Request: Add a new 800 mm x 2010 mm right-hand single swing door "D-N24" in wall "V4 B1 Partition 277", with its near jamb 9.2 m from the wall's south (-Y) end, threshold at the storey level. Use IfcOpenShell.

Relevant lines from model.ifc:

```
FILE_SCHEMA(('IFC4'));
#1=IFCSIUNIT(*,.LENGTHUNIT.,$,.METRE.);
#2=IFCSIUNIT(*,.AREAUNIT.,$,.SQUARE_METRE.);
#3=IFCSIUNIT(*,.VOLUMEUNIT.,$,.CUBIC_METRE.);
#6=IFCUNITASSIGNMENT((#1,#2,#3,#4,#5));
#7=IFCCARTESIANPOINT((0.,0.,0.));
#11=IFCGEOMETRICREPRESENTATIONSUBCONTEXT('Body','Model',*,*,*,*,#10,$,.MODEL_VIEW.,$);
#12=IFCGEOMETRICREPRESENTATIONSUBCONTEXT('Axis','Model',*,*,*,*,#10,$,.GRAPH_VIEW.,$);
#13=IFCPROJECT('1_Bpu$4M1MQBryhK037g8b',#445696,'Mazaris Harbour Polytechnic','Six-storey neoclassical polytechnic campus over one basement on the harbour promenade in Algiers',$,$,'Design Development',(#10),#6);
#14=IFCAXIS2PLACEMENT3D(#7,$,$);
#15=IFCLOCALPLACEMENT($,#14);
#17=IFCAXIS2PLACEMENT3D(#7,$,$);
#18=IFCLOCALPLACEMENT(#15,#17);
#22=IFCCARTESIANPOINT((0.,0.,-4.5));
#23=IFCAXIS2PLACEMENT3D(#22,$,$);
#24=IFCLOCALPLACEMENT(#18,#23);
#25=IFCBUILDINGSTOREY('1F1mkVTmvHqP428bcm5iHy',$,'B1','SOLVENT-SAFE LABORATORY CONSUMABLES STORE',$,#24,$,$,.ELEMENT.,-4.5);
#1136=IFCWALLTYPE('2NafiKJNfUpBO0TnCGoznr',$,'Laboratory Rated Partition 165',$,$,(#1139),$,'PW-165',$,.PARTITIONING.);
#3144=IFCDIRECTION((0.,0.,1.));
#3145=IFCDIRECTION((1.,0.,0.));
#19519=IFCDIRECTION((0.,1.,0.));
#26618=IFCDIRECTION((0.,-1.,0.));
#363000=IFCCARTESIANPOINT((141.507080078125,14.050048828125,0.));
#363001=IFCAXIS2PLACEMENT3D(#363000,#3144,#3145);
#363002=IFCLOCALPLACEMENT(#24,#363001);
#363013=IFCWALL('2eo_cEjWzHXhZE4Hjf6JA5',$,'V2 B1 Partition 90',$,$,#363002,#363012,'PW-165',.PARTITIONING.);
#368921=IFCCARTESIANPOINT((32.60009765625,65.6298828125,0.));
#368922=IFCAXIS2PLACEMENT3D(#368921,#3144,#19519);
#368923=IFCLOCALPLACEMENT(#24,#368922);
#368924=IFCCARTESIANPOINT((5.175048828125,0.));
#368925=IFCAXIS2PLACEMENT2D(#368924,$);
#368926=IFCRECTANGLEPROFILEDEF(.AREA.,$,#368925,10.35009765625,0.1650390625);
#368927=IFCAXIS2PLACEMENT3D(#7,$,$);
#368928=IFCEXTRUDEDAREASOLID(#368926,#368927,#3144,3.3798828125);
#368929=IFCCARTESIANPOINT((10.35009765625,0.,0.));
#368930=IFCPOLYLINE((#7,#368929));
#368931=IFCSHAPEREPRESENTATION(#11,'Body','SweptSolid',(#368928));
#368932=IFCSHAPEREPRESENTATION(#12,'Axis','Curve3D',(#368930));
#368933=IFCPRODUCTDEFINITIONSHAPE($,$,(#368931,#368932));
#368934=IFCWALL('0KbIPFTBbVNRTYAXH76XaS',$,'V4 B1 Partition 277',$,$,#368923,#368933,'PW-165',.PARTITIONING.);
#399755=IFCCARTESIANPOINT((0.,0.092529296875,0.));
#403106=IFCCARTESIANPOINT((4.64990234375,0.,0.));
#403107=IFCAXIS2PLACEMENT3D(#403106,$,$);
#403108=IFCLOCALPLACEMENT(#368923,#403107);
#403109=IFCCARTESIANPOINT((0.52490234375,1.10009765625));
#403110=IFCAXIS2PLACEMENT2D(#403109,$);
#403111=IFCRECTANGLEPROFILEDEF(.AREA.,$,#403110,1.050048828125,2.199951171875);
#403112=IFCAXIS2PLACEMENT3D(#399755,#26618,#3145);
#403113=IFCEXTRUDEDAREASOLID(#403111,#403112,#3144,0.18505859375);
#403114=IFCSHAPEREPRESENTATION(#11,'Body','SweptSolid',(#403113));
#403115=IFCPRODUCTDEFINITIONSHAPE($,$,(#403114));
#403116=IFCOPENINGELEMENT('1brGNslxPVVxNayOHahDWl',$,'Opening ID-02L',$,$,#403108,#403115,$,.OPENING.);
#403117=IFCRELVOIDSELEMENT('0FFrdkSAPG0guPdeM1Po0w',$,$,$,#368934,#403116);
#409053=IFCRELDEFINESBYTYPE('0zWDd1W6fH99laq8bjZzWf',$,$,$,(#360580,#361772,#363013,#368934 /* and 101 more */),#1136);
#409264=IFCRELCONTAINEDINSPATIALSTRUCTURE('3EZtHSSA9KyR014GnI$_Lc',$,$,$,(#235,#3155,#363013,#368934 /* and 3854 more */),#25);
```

```python
import numpy as np
import ifcopenshell
import ifcopenshell.api.feature
import ifcopenshell.api.geometry
import ifcopenshell.api.root
import ifcopenshell.api.spatial
import ifcopenshell.geom
import ifcopenshell.util.element
import ifcopenshell.util.placement
import ifcopenshell.util.representation
import ifcopenshell.util.shape
import ifcopenshell.util.unit

model = ifcopenshell.open("model.ifc")
unit_scale = ifcopenshell.util.unit.calculate_unit_scale(model)
settings = ifcopenshell.geom.settings()


def volume(element):
    """Net volume in cubic metres, openings subtracted."""
    shape = ifcopenshell.geom.create_shape(settings, element)
    return ifcopenshell.util.shape.get_volume(shape.geometry)


wall = model.by_id(368934)
storey = ifcopenshell.util.element.get_container(wall, ifc_class="IfcBuildingStorey")
context = ifcopenshell.util.representation.get_context(model, "Model", "Body", "MODEL_VIEW")
before = volume(wall)

width, height, from_end, sill = 0.8, 2.01, 9.2, 0.0  # metres

# The wall runs along its own X axis, and the end named is its -X end.
wall_shape = ifcopenshell.geom.create_shape(settings, wall)
x, y, z = ifcopenshell.util.shape.get_vertices(wall_shape.geometry).T
start = x.min() + from_end
face, thickness = float(y.min()), float(y.max() - y.min())
wall_matrix = ifcopenshell.util.placement.get_local_placement(wall.ObjectPlacement)
level = ifcopenshell.util.placement.get_local_placement(storey.ObjectPlacement)[2, 3]


def in_wall(x, y):
    """Placement at x, y metres in the wall's axes, at sill height."""
    matrix = wall_matrix.copy()
    matrix[:, 3] = wall_matrix @ np.array([x / unit_scale, y / unit_scale, 0.0, 1.0])
    matrix[2, 3] = level + sill / unit_scale
    return matrix


# Opening: a box that overshoots both wall faces by 50 mm.
opening = ifcopenshell.api.root.create_entity(model, ifc_class="IfcOpeningElement", predefined_type="OPENING")
box = ifcopenshell.api.geometry.add_wall_representation(
    model, context=context, length=width, height=height, thickness=thickness + 0.1
)
ifcopenshell.api.geometry.assign_representation(model, product=opening, representation=box)
ifcopenshell.api.geometry.edit_object_placement(model, product=opening, matrix=in_wall(start, face - 0.05), is_si=False)
ifcopenshell.api.feature.add_feature(model, feature=opening, element=wall)

door = ifcopenshell.api.root.create_entity(model, ifc_class="IfcDoor", name="D-N24", predefined_type="DOOR")
door.OverallWidth, door.OverallHeight = width / unit_scale, height / unit_scale
door.OperationType = "SINGLE_SWING_RIGHT"
body = ifcopenshell.api.geometry.add_door_representation(
    model,
    context=context,
    overall_width=door.OverallWidth,
    overall_height=door.OverallHeight,
    operation_type="SINGLE_SWING_RIGHT",
    lining_properties={"LiningDepth": thickness / unit_scale, "ThresholdDepth": thickness / unit_scale},
)
ifcopenshell.api.geometry.assign_representation(model, product=door, representation=body)
ifcopenshell.api.spatial.assign_container(model, products=[door], relating_structure=storey)
ifcopenshell.api.feature.add_filling(model, opening=opening, element=door)

# The lining spans the wall, so the door starts at the wall face.
ifcopenshell.api.geometry.edit_object_placement(model, product=door, matrix=in_wall(start, face), is_si=False)

after = volume(wall)

print(f"wall volume {before:.3f} -> {after:.3f} m3")

model.write("model_v2.ifc")
```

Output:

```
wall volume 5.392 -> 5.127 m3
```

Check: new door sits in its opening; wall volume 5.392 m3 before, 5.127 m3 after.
